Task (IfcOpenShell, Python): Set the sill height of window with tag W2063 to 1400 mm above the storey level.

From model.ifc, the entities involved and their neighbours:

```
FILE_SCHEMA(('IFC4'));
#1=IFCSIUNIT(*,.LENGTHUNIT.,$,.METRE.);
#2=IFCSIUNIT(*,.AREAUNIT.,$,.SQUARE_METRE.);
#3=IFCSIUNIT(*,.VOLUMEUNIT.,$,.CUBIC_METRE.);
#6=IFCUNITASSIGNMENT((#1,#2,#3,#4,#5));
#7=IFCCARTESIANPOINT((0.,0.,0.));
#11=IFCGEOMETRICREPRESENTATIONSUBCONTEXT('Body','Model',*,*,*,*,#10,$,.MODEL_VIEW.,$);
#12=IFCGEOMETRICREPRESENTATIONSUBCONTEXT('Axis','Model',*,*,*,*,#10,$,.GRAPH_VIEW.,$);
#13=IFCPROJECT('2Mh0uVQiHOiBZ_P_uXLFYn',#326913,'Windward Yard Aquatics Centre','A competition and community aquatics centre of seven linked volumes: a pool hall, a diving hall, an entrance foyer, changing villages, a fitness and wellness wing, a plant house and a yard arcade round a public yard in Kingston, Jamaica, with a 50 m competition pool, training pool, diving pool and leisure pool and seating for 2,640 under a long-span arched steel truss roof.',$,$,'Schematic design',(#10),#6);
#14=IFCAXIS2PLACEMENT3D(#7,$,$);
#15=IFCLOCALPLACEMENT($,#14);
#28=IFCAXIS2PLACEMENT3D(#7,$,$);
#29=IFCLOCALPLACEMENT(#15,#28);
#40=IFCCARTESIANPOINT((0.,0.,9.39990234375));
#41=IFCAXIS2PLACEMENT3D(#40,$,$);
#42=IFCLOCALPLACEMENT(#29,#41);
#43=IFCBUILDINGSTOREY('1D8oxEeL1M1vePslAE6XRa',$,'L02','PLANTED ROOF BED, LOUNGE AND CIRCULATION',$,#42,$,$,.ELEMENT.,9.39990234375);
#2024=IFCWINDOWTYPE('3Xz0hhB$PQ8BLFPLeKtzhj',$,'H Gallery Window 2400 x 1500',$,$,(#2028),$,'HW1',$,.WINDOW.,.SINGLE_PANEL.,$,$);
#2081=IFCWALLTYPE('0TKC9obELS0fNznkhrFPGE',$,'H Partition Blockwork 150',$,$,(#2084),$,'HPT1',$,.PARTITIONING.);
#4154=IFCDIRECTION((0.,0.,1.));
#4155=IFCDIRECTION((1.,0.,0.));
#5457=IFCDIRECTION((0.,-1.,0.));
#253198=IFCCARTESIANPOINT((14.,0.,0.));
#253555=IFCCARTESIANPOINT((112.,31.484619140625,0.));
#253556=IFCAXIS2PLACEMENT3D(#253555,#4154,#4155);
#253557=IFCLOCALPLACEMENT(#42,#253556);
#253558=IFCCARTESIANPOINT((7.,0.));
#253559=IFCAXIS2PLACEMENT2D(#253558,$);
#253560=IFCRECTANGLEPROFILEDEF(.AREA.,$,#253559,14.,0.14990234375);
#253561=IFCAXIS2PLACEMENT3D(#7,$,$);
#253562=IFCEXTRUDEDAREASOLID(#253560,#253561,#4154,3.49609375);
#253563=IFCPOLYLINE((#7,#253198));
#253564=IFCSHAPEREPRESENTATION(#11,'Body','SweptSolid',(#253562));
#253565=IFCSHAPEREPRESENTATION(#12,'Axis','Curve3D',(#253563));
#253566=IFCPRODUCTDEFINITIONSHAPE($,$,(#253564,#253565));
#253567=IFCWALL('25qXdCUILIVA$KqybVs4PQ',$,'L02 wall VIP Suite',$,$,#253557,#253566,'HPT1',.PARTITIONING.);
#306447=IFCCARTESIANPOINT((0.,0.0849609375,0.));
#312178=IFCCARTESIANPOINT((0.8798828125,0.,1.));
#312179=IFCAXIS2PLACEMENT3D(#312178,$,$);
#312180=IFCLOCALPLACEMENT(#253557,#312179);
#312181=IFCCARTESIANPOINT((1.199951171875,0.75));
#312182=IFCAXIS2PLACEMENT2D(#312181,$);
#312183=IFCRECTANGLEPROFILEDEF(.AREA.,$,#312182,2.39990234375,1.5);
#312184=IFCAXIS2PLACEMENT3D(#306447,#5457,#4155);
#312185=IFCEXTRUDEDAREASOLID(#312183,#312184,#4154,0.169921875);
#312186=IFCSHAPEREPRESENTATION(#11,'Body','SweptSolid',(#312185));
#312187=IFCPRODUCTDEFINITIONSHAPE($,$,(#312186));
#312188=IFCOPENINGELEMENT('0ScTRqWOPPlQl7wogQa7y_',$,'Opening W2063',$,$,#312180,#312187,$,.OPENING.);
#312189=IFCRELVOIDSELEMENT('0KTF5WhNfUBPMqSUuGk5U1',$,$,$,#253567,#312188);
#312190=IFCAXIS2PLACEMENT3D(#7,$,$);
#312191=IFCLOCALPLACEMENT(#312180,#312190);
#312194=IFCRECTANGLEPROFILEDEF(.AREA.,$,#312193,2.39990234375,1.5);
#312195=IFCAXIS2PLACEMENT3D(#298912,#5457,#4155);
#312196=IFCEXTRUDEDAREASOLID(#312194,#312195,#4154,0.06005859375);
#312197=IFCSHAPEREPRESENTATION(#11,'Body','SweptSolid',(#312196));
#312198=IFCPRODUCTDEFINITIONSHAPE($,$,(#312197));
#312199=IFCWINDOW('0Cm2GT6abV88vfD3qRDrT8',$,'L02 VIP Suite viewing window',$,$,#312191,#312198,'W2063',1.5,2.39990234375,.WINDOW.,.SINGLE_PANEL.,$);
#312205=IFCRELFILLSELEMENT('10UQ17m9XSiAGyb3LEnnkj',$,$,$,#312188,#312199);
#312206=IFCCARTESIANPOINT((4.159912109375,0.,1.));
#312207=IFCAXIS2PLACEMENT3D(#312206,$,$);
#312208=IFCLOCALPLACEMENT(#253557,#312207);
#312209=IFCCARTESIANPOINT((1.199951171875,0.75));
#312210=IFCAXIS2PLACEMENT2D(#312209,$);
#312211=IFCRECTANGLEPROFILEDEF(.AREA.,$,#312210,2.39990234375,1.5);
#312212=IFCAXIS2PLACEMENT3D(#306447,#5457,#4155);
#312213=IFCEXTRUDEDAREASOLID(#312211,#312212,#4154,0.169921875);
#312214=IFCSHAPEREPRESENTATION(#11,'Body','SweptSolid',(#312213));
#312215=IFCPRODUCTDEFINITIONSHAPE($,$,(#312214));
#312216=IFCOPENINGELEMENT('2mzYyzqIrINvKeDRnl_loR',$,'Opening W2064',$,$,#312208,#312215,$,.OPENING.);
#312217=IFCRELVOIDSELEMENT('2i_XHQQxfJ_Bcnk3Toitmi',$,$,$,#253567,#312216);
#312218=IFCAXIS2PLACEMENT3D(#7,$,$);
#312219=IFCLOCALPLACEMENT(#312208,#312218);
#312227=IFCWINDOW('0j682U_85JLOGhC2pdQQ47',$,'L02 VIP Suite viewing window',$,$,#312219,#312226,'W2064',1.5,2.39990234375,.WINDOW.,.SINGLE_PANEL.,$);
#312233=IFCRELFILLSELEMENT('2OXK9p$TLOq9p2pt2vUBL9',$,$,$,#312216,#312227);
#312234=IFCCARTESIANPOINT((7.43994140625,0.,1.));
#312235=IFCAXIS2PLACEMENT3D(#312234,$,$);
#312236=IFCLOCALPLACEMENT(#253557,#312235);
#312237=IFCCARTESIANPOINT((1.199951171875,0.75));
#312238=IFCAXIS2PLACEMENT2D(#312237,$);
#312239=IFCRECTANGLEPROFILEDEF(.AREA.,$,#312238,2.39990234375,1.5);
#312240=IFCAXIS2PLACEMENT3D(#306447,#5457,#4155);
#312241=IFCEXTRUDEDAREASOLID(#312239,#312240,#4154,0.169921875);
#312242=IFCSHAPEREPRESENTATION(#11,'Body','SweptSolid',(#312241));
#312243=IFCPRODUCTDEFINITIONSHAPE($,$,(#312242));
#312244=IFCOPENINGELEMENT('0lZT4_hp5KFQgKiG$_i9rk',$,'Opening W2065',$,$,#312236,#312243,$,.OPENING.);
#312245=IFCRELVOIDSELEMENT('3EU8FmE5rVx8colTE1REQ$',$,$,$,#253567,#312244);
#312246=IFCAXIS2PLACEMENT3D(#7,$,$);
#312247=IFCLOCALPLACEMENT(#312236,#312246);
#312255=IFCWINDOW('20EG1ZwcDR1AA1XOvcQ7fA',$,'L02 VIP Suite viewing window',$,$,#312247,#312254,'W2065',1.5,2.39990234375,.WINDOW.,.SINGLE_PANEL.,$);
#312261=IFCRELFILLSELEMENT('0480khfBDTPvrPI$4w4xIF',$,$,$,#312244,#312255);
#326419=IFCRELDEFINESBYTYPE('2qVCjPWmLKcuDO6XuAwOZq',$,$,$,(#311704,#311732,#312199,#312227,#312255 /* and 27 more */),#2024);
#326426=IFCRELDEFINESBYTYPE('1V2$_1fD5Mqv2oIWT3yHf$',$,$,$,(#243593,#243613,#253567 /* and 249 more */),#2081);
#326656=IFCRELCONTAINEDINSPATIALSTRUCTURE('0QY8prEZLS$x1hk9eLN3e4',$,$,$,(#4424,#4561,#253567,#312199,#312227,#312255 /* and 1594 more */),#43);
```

```python
import numpy as np
import ifcopenshell
import ifcopenshell.api.geometry
import ifcopenshell.geom
import ifcopenshell.util.element
import ifcopenshell.util.placement
import ifcopenshell.util.shape
import ifcopenshell.util.unit

model = ifcopenshell.open("model.ifc")
unit_scale = ifcopenshell.util.unit.calculate_unit_scale(model)

window = model.by_id(312199)
opening = window.FillsVoids[0].RelatingOpeningElement
storey = ifcopenshell.util.element.get_container(window, ifc_class="IfcBuildingStorey")
level = ifcopenshell.util.placement.get_local_placement(storey.ObjectPlacement)[2, 3]

# The opening's origin need not be at the sill, so measure its lowest point.
shape = ifcopenshell.geom.create_shape(ifcopenshell.geom.settings(), opening)
bottom = ifcopenshell.util.shape.get_shape_bottom_elevation(shape, shape.geometry) / unit_scale
dz = level + 1.4 - bottom

shift = np.array([0.0, 0.0, dz])
# The window is placed relative to its opening, so it follows when the opening moves.
matrix = ifcopenshell.util.placement.get_local_placement(opening.ObjectPlacement)
matrix[:3, 3] += shift
ifcopenshell.api.geometry.edit_object_placement(
    model, product=opening, matrix=matrix, is_si=False, should_transform_children=True
)

print(f"moved by {dz * unit_scale:+.3f} m")

model.write("model_v2.ifc")
```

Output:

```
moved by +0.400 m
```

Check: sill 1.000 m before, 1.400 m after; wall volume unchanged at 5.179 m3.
